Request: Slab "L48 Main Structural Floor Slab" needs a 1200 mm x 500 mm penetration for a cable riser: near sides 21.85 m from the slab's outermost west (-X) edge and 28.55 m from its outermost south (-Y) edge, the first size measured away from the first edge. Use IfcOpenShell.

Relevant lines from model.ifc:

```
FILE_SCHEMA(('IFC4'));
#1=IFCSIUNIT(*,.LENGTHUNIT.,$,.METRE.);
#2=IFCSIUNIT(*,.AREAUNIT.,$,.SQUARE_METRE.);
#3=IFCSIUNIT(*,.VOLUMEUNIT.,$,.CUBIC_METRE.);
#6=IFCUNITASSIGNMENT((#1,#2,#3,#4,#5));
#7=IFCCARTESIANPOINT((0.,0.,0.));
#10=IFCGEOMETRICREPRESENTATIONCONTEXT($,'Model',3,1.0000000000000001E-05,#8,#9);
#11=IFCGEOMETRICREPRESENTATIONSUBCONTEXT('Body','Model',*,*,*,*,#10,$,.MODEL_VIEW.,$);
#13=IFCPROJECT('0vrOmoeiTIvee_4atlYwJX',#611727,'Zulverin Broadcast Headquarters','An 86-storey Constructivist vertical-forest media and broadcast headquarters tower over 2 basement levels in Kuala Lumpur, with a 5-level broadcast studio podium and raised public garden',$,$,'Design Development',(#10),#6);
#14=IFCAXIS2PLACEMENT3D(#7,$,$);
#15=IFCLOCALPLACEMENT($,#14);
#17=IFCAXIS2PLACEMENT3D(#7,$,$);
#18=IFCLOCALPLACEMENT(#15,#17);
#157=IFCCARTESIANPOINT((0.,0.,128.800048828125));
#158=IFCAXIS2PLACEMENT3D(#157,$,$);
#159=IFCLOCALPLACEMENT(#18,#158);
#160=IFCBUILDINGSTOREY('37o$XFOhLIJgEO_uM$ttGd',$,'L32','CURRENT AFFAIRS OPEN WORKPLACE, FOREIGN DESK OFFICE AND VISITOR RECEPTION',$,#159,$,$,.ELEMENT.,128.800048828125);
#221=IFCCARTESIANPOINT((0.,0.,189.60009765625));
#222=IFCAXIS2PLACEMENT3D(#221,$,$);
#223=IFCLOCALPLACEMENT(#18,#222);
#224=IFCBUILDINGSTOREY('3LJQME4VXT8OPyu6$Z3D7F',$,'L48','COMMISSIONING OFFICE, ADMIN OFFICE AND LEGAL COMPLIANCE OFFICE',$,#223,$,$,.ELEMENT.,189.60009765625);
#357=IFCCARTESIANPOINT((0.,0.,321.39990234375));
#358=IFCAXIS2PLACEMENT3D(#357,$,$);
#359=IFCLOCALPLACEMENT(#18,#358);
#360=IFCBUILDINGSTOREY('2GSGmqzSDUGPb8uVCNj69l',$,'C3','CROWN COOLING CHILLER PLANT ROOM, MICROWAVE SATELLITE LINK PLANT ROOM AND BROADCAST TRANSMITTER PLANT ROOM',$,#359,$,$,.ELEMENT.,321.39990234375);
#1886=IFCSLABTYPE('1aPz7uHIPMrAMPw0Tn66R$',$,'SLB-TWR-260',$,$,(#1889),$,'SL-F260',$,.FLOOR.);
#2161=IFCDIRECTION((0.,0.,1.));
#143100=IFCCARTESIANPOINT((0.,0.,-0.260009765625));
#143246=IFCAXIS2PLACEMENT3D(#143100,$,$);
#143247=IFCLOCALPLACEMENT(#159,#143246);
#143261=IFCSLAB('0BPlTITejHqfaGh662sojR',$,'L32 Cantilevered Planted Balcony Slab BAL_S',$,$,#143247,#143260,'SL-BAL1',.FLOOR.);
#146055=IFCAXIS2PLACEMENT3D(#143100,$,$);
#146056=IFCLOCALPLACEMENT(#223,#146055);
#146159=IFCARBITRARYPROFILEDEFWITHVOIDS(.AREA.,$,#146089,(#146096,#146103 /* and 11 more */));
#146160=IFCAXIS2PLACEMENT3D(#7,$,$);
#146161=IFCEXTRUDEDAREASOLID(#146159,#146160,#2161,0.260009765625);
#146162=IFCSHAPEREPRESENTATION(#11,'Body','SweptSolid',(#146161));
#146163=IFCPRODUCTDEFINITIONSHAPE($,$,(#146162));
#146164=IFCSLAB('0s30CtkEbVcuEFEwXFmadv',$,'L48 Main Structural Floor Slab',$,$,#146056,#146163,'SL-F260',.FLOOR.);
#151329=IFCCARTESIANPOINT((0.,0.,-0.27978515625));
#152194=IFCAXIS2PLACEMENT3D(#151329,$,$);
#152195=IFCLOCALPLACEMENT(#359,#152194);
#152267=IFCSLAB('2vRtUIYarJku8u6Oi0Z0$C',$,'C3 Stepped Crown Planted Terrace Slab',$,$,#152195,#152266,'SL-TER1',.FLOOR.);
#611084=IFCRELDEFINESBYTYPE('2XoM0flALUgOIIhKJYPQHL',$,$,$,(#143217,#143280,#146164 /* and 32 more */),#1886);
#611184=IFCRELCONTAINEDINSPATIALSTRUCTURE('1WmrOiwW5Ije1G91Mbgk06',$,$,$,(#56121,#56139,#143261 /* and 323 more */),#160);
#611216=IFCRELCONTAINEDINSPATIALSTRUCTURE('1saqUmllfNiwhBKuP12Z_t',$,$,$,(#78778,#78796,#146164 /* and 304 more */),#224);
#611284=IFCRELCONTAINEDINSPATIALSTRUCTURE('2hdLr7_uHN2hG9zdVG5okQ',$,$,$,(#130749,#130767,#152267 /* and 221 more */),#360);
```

```python
import numpy as np
import ifcopenshell
import ifcopenshell.api.feature
import ifcopenshell.api.geometry
import ifcopenshell.api.root
import ifcopenshell.geom
import ifcopenshell.util.placement
import ifcopenshell.util.representation
import ifcopenshell.util.shape
import ifcopenshell.util.unit

model = ifcopenshell.open("model.ifc")
unit_scale = ifcopenshell.util.unit.calculate_unit_scale(model)
settings = ifcopenshell.geom.settings()


def volume(element):
    """Net volume in cubic metres, openings subtracted."""
    shape = ifcopenshell.geom.create_shape(settings, element)
    return ifcopenshell.util.shape.get_volume(shape.geometry)


slab = model.by_guid("0s30CtkEbVcuEFEwXFmadv")
before = volume(slab)

# Extent in the slab's own axes, in metres. The edges named are its -X and -Y sides.
slab_shape = ifcopenshell.geom.create_shape(settings, slab)
vertices = ifcopenshell.util.shape.get_vertices(slab_shape.geometry)
x_min, y_min, bottom = vertices.min(axis=0)
top = vertices[:, 2].max()

opening = ifcopenshell.api.root.create_entity(model, ifc_class="IfcOpeningElement", name="Cable riser opening", predefined_type="OPENING")
context = ifcopenshell.util.representation.get_context(model, "Model", "Body", "MODEL_VIEW")
width, depth = 1.2, 0.5
outline = [(0.0, 0.0), (width, 0.0), (width, depth), (0.0, depth), (0.0, 0.0)]
# Overshoot both faces by 50 mm so the cut is clean.
shape = ifcopenshell.api.geometry.add_slab_representation(
    model, context=context, depth=top - bottom + 0.1, polyline=outline
)
ifcopenshell.api.geometry.assign_representation(model, product=opening, representation=shape)

matrix = ifcopenshell.util.placement.get_local_placement(slab.ObjectPlacement)
matrix[:, 3] = matrix @ np.append(np.array([x_min + 21.85, y_min + 28.55, bottom - 0.05]) / unit_scale, 1.0)
ifcopenshell.api.geometry.edit_object_placement(model, product=opening, matrix=matrix, is_si=False)
ifcopenshell.api.feature.add_feature(model, feature=opening, element=slab)

after = volume(slab)

print(f"slab volume {before:.3f} -> {after:.3f} m3")

model.write("model_edited.ifc")
```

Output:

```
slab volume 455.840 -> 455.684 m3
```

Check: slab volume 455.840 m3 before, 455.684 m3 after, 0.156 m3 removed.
